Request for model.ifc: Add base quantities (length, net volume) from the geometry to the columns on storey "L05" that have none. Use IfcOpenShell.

First a look at what the model holds.

```python
import ifcopenshell
import ifcopenshell.util.element
import ifcopenshell.util.unit

model = ifcopenshell.open("model.ifc")
print(model.schema)
for unit_type in ("LENGTHUNIT", "AREAUNIT", "VOLUMEUNIT"):
    print(unit_type, ifcopenshell.util.unit.calculate_unit_scale(model, unit_type))
storey = next(s for s in model.by_type("IfcBuildingStorey") if s.Name == "L05")
columns = [e for e in ifcopenshell.util.element.get_decomposition(storey) if e.is_a("IfcColumn")]
for e in sorted(columns, key=lambda e: e.id()):
    print(e.id(), e.is_a(), e.Name, list(ifcopenshell.util.element.get_psets(e, qtos_only=True)), sep=" | ")
```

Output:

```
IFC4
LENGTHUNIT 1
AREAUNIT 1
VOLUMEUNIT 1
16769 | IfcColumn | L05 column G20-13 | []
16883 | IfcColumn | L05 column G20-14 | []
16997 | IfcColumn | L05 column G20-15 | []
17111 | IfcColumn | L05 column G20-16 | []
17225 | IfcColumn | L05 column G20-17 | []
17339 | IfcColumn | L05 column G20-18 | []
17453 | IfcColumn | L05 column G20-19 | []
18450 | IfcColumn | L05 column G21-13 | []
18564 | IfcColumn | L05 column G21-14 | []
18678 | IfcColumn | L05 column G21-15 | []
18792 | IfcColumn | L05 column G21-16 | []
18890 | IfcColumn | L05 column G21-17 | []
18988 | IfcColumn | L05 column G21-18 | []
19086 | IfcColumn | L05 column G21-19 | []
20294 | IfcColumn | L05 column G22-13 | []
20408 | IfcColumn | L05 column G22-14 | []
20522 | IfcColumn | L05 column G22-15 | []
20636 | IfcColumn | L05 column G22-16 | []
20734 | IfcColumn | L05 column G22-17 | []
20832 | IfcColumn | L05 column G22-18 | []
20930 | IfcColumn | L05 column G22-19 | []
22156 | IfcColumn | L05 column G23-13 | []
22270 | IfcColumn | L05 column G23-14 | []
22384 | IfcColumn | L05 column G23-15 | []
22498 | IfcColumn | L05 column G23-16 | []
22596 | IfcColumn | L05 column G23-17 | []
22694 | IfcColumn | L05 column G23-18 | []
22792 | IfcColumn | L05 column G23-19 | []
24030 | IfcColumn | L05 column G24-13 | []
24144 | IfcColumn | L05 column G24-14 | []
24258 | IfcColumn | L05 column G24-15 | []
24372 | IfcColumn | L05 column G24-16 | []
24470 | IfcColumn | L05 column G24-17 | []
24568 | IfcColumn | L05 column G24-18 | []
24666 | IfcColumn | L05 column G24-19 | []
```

```python
import ifcopenshell
import ifcopenshell.api.pset
import ifcopenshell.geom
import ifcopenshell.util.element
import ifcopenshell.util.shape
import ifcopenshell.util.unit

model = ifcopenshell.open("model.ifc")
unit_scale = ifcopenshell.util.unit.calculate_unit_scale(model)
volume_scale = ifcopenshell.util.unit.calculate_unit_scale(model, "VOLUMEUNIT")
settings = ifcopenshell.geom.settings()

storey = next(s for s in model.by_type("IfcBuildingStorey") if s.Name == "L05")
columns = [e for e in ifcopenshell.util.element.get_decomposition(storey) if e.is_a("IfcColumn")]

for e in sorted(columns, key=lambda e: e.id()):
    if ifcopenshell.util.element.get_psets(e, qtos_only=True, should_inherit=False):
        continue
    # Geometry comes back in metres, in the element's own axes.
    shape = ifcopenshell.geom.create_shape(settings, e)
    values = {
        "Length": ifcopenshell.util.shape.get_z(shape.geometry) / unit_scale,
        "NetVolume": ifcopenshell.util.shape.get_volume(shape.geometry) / volume_scale,
    }
    qto = ifcopenshell.api.pset.add_qto(model, product=e, name="Qto_ColumnBaseQuantities")
    ifcopenshell.api.pset.edit_qto(model, qto=qto, properties=values)
    print(e.id(), {k: round(v, 3) for k, v in values.items()})

model.write("model_edited.ifc")
```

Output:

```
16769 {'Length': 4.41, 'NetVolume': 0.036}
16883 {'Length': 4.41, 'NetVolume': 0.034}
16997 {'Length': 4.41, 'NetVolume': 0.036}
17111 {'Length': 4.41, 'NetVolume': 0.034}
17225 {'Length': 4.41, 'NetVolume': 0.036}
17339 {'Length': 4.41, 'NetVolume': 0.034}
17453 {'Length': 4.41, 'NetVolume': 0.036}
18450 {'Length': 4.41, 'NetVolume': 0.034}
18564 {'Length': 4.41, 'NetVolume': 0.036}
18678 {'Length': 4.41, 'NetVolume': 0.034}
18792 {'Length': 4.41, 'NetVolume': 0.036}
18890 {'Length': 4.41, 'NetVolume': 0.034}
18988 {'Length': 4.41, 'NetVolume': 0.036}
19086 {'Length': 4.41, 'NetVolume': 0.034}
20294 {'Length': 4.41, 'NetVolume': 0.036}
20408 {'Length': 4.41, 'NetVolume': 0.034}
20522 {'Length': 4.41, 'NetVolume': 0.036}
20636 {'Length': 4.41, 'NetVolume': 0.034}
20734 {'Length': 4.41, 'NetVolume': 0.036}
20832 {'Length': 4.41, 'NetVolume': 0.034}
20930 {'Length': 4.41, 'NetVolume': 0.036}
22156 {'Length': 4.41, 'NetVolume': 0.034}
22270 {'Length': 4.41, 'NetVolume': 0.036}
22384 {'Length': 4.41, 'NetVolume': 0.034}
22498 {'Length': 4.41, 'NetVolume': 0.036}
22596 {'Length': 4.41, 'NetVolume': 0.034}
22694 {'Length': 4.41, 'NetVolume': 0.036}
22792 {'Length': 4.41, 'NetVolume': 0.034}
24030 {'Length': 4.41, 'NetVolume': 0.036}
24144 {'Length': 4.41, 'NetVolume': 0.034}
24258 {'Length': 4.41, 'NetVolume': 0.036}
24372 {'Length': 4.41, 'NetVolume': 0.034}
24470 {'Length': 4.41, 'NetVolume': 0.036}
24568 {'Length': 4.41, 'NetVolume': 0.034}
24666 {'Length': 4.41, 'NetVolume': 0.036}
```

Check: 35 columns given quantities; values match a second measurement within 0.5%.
